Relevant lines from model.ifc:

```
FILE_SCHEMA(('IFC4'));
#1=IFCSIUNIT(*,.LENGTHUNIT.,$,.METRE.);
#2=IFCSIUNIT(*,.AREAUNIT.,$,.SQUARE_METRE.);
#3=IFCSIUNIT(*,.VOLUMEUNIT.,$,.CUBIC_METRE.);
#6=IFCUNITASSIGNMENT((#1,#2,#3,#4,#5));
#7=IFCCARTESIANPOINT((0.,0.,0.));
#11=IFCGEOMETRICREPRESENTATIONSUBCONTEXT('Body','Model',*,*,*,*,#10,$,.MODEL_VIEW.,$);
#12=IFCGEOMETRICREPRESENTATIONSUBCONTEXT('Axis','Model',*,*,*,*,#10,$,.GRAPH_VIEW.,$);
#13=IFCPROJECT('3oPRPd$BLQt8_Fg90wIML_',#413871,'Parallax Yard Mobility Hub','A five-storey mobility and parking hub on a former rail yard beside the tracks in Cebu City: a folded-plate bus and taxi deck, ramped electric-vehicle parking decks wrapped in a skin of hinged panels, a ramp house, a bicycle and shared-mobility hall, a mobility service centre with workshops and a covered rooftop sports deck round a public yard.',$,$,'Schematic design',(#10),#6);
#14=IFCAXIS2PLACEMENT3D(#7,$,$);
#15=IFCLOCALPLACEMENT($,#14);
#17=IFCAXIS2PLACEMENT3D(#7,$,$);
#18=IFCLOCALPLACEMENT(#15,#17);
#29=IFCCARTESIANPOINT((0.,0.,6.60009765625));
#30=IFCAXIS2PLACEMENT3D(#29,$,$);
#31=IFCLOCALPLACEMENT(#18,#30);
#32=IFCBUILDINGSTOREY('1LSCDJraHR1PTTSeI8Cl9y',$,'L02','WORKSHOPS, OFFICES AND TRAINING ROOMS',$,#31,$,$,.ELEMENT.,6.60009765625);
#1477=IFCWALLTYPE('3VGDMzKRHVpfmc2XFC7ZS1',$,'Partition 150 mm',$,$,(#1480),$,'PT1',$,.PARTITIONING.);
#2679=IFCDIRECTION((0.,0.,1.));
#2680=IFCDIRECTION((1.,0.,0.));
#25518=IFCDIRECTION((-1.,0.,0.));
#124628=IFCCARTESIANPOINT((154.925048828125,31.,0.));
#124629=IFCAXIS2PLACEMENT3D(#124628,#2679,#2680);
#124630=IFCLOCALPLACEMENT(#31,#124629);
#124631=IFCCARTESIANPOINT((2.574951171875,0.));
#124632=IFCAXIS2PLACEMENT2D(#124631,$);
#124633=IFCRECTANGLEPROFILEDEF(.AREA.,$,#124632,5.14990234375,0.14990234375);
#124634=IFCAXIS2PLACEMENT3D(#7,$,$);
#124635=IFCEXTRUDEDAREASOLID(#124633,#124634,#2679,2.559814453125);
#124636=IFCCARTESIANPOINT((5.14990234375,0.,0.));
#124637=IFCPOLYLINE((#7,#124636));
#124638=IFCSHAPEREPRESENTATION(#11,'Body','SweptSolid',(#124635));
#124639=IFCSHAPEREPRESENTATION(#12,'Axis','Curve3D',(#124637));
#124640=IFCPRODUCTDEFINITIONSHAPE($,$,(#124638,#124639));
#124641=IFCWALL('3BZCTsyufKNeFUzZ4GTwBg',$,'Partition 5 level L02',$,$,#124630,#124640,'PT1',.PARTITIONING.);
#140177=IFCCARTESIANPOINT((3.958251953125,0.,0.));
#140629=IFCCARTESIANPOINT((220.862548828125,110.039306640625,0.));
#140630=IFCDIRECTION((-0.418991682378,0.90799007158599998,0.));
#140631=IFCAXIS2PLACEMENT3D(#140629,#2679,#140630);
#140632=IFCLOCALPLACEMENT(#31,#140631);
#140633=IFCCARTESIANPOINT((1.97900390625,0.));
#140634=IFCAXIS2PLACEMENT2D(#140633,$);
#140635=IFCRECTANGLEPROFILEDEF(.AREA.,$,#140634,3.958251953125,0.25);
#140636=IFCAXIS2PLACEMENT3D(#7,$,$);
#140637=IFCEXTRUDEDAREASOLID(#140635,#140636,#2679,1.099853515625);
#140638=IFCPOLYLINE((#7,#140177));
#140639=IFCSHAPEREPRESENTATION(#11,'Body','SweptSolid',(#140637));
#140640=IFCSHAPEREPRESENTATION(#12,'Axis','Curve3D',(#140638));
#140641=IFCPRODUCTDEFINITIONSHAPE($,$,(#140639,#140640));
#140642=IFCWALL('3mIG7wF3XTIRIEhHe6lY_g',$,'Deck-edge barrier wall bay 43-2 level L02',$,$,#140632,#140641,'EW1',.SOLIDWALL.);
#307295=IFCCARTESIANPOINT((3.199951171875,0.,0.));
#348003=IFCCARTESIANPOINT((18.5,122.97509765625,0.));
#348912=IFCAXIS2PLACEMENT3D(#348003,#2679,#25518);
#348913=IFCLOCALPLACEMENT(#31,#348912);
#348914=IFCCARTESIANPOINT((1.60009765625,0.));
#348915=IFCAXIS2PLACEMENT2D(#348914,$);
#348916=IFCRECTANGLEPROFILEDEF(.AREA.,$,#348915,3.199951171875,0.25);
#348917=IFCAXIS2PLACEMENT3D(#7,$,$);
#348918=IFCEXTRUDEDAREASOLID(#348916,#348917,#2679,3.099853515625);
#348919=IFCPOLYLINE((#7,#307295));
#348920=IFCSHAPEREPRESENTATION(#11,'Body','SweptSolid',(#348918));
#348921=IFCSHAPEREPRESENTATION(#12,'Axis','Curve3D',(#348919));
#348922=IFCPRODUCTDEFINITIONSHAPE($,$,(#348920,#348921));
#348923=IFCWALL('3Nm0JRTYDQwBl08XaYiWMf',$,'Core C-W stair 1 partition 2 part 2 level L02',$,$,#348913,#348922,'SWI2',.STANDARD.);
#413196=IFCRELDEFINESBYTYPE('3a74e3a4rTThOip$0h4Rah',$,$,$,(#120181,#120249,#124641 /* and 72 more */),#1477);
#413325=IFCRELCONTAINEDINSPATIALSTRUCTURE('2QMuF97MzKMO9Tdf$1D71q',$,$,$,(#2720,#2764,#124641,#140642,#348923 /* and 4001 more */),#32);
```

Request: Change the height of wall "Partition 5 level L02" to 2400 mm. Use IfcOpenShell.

```python
import ifcopenshell
import ifcopenshell.geom
import ifcopenshell.util.representation
import ifcopenshell.util.shape
import ifcopenshell.util.unit

model = ifcopenshell.open("model.ifc")
unit_scale = ifcopenshell.util.unit.calculate_unit_scale(model)
settings = ifcopenshell.geom.settings()


def volume(element):
    """Net volume in cubic metres, openings subtracted."""
    shape = ifcopenshell.geom.create_shape(settings, element)
    return ifcopenshell.util.shape.get_volume(shape.geometry)


wall = model.by_id(124641)
before = volume(wall)

body = ifcopenshell.util.representation.get_representation(wall, "Model", "Body")
solid = body.Items[0]
old_height = solid.Depth
solid.Depth = 2.4 / unit_scale
after = volume(wall)

print(f"height {old_height:g} -> {solid.Depth:g}, volume {before:.3f} -> {after:.3f} m3")

model.write("model_updated.ifc")
```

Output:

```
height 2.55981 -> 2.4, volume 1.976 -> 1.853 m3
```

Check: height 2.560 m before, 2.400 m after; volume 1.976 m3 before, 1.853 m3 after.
